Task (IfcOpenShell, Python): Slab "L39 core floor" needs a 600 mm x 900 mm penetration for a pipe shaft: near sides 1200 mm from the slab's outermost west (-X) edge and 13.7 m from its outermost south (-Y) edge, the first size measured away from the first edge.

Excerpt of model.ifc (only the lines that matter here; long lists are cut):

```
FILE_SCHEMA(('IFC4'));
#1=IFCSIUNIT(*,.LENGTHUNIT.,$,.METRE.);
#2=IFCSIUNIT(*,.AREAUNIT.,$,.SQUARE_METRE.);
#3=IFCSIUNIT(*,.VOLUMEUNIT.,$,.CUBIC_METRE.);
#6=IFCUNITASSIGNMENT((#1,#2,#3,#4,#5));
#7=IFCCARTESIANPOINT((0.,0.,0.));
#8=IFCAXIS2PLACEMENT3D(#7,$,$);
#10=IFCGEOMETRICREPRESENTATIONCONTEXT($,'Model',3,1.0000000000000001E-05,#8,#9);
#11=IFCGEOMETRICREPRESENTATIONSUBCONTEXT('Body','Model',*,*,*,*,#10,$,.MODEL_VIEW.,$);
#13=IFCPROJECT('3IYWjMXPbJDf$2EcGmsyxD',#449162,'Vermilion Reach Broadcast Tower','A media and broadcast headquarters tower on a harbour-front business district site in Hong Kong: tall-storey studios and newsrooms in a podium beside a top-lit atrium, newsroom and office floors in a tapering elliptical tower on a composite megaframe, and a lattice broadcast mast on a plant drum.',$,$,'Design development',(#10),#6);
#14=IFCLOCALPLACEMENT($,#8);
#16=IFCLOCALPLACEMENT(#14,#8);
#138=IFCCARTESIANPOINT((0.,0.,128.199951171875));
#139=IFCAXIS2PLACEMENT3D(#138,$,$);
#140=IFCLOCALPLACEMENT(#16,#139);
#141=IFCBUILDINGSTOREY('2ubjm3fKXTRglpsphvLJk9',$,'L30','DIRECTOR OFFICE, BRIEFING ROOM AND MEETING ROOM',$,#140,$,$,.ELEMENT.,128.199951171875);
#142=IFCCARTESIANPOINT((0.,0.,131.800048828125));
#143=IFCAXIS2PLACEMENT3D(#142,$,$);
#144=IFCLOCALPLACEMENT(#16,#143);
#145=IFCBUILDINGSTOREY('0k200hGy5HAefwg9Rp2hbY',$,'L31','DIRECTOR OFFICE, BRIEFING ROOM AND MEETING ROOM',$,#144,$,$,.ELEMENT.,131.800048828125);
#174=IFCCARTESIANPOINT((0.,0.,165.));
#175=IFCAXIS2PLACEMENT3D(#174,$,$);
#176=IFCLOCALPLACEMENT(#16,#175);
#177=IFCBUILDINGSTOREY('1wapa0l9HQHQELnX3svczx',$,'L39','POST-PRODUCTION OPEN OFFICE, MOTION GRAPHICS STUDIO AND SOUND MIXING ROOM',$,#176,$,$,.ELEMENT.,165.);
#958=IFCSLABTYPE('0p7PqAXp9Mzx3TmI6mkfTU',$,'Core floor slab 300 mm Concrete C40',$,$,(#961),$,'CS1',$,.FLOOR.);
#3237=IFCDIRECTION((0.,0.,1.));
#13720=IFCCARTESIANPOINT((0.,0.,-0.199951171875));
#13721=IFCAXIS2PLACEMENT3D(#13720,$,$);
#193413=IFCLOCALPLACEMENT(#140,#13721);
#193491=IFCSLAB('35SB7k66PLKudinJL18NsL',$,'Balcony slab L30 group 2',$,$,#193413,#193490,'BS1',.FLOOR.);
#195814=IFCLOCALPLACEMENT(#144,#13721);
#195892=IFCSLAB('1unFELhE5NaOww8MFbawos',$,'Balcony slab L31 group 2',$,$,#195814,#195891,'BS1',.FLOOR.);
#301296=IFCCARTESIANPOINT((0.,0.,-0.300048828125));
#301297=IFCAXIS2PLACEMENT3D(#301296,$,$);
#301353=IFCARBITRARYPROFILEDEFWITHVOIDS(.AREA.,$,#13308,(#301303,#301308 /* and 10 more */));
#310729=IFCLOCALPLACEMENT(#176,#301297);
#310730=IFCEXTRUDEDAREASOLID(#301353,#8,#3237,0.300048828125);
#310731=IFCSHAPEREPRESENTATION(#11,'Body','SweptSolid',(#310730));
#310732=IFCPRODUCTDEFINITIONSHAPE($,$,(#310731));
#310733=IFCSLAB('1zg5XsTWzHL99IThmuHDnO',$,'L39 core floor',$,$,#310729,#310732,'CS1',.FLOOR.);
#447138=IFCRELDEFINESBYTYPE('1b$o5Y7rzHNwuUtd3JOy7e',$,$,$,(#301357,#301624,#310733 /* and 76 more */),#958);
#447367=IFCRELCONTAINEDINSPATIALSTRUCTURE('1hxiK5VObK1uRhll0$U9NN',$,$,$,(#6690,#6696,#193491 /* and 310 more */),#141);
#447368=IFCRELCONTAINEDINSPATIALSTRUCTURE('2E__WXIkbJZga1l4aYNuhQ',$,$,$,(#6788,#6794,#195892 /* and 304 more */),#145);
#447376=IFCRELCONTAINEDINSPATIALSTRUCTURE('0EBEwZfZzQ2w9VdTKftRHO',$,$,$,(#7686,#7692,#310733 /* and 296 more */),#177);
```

```python
import numpy as np
import ifcopenshell
import ifcopenshell.api.feature
import ifcopenshell.api.geometry
import ifcopenshell.api.root
import ifcopenshell.geom
import ifcopenshell.util.placement
import ifcopenshell.util.representation
import ifcopenshell.util.shape
import ifcopenshell.util.unit

model = ifcopenshell.open("model.ifc")
unit_scale = ifcopenshell.util.unit.calculate_unit_scale(model)
settings = ifcopenshell.geom.settings()


def volume(element):
    """Net volume in cubic metres, openings subtracted."""
    shape = ifcopenshell.geom.create_shape(settings, element)
    return ifcopenshell.util.shape.get_volume(shape.geometry)


slab = model.by_id(310733)
before = volume(slab)

# Extent in the slab's own axes, in metres. The edges named are its -X and -Y sides.
slab_shape = ifcopenshell.geom.create_shape(settings, slab)
vertices = ifcopenshell.util.shape.get_vertices(slab_shape.geometry)
x_min, y_min, bottom = vertices.min(axis=0)
top = vertices[:, 2].max()

opening = ifcopenshell.api.root.create_entity(model, ifc_class="IfcOpeningElement", name="Pipe shaft opening", predefined_type="OPENING")
context = ifcopenshell.util.representation.get_context(model, "Model", "Body", "MODEL_VIEW")
width, depth = 0.6, 0.9
outline = [(0.0, 0.0), (width, 0.0), (width, depth), (0.0, depth), (0.0, 0.0)]
# Overshoot both faces by 50 mm so the cut is clean.
shape = ifcopenshell.api.geometry.add_slab_representation(
    model, context=context, depth=top - bottom + 0.1, polyline=outline
)
ifcopenshell.api.geometry.assign_representation(model, product=opening, representation=shape)

matrix = ifcopenshell.util.placement.get_local_placement(slab.ObjectPlacement)
matrix[:, 3] = matrix @ np.append(np.array([x_min + 1.2, y_min + 13.7, bottom - 0.05]) / unit_scale, 1.0)
ifcopenshell.api.geometry.edit_object_placement(model, product=opening, matrix=matrix, is_si=False)
ifcopenshell.api.feature.add_feature(model, feature=opening, element=slab)

after = volume(slab)

print(f"slab volume {before:.3f} -> {after:.3f} m3")

model.write("model_edited.ifc")
```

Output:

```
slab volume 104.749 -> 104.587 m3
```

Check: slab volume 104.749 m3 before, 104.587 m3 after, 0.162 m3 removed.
